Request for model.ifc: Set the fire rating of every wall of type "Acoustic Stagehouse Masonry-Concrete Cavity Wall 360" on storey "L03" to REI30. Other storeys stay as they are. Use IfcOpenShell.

First a look at what the model holds.

```python
import ifcopenshell
import ifcopenshell.util.element

model = ifcopenshell.open("model.ifc")
print(model.schema)
storey = next(s for s in model.by_type("IfcBuildingStorey") if s.Name == "L03")
walls = [e for e in ifcopenshell.util.element.get_decomposition(storey) if e.is_a("IfcWall")]
seen = {}
for e in walls:
    element_type = ifcopenshell.util.element.get_type(e)
    key = (element_type.Name if element_type != e and element_type else None, ifcopenshell.util.element.get_pset(e, "Pset_WallCommon", "FireRating"))
    seen[key] = seen.get(key, 0) + 1
for (name, value), count in sorted(seen.items(), key=str):
    print(count, "x", name, "|", value)
```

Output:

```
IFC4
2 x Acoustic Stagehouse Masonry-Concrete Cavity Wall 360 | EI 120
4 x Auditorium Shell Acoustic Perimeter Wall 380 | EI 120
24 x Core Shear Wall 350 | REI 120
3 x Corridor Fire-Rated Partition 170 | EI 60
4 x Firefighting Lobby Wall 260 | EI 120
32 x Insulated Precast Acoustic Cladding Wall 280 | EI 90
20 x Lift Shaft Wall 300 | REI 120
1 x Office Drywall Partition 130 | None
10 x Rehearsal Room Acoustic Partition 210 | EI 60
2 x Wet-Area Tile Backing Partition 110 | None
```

```python
import ifcopenshell
import ifcopenshell.api.pset
import ifcopenshell.util.element

model = ifcopenshell.open("model.ifc")

storey = next(s for s in model.by_type("IfcBuildingStorey") if s.Name == "L03")
walls = [e for e in ifcopenshell.util.element.get_decomposition(storey) if e.is_a("IfcWall")]

count = 0
for e in walls:
    element_type = ifcopenshell.util.element.get_type(e)
    if element_type in (None, e) or element_type.Name != "Acoustic Stagehouse Masonry-Concrete Cavity Wall 360":
        continue
    # add_pset returns the element's existing set when there is one.
    pset = ifcopenshell.api.pset.add_pset(model, product=e, name="Pset_WallCommon")
    ifcopenshell.api.pset.edit_pset(model, pset=pset, properties={"FireRating": "REI30"})
    count += 1

print(count, "walls updated")

model.write("model_v2.ifc")
```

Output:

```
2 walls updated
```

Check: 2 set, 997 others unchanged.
